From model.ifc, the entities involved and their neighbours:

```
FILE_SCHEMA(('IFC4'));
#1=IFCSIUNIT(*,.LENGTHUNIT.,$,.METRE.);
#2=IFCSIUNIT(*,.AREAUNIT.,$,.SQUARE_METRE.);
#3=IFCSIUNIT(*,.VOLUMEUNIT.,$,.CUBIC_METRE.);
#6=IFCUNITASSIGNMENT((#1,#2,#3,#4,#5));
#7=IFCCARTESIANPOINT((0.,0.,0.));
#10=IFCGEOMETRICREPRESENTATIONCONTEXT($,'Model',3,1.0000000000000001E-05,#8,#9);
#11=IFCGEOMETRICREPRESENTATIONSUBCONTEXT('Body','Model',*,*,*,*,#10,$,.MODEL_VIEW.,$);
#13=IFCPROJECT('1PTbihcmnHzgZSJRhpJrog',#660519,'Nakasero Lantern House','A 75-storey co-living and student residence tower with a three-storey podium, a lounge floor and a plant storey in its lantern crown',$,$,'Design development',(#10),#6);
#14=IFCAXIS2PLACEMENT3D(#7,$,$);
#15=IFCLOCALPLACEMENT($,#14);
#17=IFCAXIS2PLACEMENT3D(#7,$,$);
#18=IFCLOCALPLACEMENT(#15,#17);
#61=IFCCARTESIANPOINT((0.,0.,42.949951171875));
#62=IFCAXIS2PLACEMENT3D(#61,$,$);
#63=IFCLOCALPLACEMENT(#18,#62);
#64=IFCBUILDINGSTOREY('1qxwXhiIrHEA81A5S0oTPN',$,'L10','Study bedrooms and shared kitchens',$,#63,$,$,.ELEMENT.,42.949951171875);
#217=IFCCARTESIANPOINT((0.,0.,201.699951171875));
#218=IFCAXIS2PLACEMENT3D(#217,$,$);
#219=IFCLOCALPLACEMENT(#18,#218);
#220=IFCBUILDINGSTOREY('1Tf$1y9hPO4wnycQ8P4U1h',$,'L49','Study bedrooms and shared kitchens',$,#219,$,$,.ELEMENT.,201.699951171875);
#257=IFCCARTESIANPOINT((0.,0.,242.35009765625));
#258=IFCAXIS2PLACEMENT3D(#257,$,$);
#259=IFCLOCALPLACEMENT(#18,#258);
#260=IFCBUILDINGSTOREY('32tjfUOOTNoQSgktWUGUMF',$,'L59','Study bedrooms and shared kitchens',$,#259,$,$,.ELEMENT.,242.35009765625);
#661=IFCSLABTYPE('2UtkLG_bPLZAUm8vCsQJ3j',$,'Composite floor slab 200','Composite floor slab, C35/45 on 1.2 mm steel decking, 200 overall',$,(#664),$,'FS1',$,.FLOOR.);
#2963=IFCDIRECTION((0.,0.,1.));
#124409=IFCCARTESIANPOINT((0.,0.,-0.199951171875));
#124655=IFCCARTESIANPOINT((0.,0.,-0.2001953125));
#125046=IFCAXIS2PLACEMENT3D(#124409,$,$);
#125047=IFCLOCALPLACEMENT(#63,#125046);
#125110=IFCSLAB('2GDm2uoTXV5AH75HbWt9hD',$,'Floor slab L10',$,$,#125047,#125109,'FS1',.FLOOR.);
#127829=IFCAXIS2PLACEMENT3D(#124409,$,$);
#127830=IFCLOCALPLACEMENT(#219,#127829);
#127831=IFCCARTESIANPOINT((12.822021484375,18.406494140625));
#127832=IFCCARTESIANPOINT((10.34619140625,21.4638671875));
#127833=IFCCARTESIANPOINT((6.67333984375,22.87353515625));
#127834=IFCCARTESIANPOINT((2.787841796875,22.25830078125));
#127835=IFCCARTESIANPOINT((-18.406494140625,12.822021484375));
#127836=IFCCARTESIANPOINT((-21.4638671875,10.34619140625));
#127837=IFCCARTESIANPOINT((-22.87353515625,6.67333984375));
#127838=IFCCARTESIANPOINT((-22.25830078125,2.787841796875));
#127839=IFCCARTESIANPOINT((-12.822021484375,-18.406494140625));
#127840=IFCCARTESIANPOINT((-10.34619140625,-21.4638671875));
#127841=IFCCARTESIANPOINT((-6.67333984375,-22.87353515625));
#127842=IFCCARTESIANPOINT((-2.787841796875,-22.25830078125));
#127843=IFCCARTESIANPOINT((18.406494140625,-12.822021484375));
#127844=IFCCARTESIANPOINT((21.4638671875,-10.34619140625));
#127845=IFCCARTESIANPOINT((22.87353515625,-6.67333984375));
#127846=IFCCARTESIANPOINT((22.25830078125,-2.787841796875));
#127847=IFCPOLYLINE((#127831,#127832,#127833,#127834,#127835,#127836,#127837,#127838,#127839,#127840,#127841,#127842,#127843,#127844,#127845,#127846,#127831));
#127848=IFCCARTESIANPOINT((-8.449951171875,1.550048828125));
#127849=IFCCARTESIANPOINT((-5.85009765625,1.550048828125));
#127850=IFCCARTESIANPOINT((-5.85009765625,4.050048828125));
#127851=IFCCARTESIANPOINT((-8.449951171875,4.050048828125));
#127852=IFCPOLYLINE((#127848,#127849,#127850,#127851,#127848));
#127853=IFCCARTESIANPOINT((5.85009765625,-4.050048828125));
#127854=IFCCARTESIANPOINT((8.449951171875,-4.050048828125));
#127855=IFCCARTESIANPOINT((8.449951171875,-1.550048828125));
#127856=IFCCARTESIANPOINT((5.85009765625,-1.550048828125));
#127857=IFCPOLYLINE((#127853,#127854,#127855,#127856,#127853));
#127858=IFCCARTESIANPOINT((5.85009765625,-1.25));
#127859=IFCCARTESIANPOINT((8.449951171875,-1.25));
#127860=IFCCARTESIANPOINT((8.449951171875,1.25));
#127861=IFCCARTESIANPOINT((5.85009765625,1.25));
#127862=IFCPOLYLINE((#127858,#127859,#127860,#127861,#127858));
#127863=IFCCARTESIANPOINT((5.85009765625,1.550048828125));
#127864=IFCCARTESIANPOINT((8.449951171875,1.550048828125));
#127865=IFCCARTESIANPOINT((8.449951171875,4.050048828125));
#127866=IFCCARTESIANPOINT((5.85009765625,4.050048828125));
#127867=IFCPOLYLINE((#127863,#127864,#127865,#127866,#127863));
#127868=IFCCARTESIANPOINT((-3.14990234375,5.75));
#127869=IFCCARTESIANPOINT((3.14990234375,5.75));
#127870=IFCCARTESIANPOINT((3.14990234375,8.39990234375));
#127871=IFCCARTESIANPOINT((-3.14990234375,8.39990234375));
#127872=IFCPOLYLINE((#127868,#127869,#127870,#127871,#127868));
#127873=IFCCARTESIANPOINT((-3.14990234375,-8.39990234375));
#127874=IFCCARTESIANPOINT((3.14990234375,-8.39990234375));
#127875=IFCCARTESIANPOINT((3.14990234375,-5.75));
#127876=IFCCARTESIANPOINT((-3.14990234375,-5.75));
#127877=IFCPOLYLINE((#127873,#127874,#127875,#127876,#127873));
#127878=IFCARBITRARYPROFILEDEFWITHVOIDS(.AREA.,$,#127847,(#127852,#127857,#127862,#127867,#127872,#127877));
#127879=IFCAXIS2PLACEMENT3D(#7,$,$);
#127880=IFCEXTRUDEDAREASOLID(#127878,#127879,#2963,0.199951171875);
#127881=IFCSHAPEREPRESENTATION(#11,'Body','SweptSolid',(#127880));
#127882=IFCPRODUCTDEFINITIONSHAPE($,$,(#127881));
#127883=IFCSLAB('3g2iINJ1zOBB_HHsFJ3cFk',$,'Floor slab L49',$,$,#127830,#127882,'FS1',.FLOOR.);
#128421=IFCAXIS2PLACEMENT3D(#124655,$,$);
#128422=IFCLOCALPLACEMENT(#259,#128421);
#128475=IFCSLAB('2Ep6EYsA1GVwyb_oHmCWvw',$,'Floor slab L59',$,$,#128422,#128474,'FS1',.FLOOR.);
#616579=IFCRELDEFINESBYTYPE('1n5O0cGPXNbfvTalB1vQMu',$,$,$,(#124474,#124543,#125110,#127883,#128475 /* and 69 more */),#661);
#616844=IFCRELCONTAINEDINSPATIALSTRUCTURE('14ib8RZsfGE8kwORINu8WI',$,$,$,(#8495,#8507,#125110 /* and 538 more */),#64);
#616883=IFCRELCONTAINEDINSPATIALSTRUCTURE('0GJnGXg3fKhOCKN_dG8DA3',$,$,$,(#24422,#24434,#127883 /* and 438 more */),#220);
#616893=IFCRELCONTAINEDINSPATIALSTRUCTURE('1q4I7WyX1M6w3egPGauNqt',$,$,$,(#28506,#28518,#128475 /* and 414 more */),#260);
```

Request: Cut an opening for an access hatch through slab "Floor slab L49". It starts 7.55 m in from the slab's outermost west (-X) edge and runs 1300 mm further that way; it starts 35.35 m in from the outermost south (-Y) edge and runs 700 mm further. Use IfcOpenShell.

```python
import numpy as np
import ifcopenshell
import ifcopenshell.api.feature
import ifcopenshell.api.geometry
import ifcopenshell.api.root
import ifcopenshell.geom
import ifcopenshell.util.placement
import ifcopenshell.util.representation
import ifcopenshell.util.shape
import ifcopenshell.util.unit

model = ifcopenshell.open("model.ifc")
unit_scale = ifcopenshell.util.unit.calculate_unit_scale(model)
settings = ifcopenshell.geom.settings()


def volume(element):
    """Net volume in cubic metres, openings subtracted."""
    shape = ifcopenshell.geom.create_shape(settings, element)
    return ifcopenshell.util.shape.get_volume(shape.geometry)


slab = model.by_guid("3g2iINJ1zOBB_HHsFJ3cFk")
before = volume(slab)

# Extent in the slab's own axes, in metres. The edges named are its -X and -Y sides.
slab_shape = ifcopenshell.geom.create_shape(settings, slab)
vertices = ifcopenshell.util.shape.get_vertices(slab_shape.geometry)
x_min, y_min, bottom = vertices.min(axis=0)
top = vertices[:, 2].max()

opening = ifcopenshell.api.root.create_entity(model, ifc_class="IfcOpeningElement", name="Access hatch opening", predefined_type="OPENING")
context = ifcopenshell.util.representation.get_context(model, "Model", "Body", "MODEL_VIEW")
width, depth = 1.3, 0.7
outline = [(0.0, 0.0), (width, 0.0), (width, depth), (0.0, depth), (0.0, 0.0)]
# Overshoot both faces by 50 mm so the cut is clean.
shape = ifcopenshell.api.geometry.add_slab_representation(
    model, context=context, depth=top - bottom + 0.1, polyline=outline
)
ifcopenshell.api.geometry.assign_representation(model, product=opening, representation=shape)

matrix = ifcopenshell.util.placement.get_local_placement(slab.ObjectPlacement)
matrix[:, 3] = matrix @ np.append(np.array([x_min + 7.55, y_min + 35.35, bottom - 0.05]) / unit_scale, 1.0)
ifcopenshell.api.geometry.edit_object_placement(model, product=opening, matrix=matrix, is_si=False)
ifcopenshell.api.feature.add_feature(model, feature=opening, element=slab)

after = volume(slab)

print(f"slab volume {before:.3f} -> {after:.3f} m3")

model.write("model_rev.ifc")
```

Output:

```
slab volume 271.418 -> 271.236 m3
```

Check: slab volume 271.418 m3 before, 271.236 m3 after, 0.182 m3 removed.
